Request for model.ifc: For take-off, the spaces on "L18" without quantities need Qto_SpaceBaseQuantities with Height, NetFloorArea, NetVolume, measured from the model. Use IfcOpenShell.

First a look at what the model holds.

```python
import ifcopenshell
import ifcopenshell.util.element
import ifcopenshell.util.unit

model = ifcopenshell.open("model.ifc")
print(model.schema)
for unit_type in ("LENGTHUNIT", "AREAUNIT", "VOLUMEUNIT"):
    print(unit_type, ifcopenshell.util.unit.calculate_unit_scale(model, unit_type))
storey = next(s for s in model.by_type("IfcBuildingStorey") if s.Name == "L18")
spaces = [e for e in ifcopenshell.util.element.get_decomposition(storey) if e.is_a("IfcSpace")]
for e in sorted(spaces, key=lambda e: e.id()):
    print(e.id(), e.is_a(), e.Name, list(ifcopenshell.util.element.get_psets(e, qtos_only=True)), sep=" | ")
```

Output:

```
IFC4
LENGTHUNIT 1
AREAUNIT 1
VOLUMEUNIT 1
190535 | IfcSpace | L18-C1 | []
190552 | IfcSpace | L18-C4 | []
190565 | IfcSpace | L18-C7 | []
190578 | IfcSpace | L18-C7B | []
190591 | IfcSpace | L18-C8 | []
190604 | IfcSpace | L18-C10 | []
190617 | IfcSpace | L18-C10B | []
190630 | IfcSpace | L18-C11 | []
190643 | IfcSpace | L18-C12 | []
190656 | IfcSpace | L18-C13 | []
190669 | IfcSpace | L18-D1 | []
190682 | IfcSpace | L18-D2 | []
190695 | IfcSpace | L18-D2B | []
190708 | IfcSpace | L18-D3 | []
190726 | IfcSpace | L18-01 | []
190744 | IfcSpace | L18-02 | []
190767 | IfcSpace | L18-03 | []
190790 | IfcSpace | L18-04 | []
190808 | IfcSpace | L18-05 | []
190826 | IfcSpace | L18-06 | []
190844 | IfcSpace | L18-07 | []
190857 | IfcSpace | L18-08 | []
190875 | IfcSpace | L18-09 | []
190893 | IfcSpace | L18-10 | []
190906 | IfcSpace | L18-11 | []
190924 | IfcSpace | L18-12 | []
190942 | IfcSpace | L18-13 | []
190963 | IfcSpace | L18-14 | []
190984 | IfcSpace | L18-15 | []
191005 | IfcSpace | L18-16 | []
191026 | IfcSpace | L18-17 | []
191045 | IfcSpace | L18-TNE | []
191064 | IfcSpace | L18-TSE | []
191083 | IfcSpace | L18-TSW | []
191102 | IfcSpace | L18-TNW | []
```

```python
import ifcopenshell
import ifcopenshell.api.pset
import ifcopenshell.geom
import ifcopenshell.util.element
import ifcopenshell.util.shape
import ifcopenshell.util.unit

model = ifcopenshell.open("model.ifc")
unit_scale = ifcopenshell.util.unit.calculate_unit_scale(model)
area_scale = ifcopenshell.util.unit.calculate_unit_scale(model, "AREAUNIT")
volume_scale = ifcopenshell.util.unit.calculate_unit_scale(model, "VOLUMEUNIT")
settings = ifcopenshell.geom.settings()

storey = next(s for s in model.by_type("IfcBuildingStorey") if s.Name == "L18")
spaces = [e for e in ifcopenshell.util.element.get_decomposition(storey) if e.is_a("IfcSpace")]

for e in sorted(spaces, key=lambda e: e.id()):
    if ifcopenshell.util.element.get_psets(e, qtos_only=True, should_inherit=False):
        continue
    # Geometry comes back in metres, in the element's own axes.
    shape = ifcopenshell.geom.create_shape(settings, e)
    values = {
        "Height": ifcopenshell.util.shape.get_z(shape.geometry) / unit_scale,
        "NetFloorArea": ifcopenshell.util.shape.get_footprint_area(shape.geometry) / area_scale,
        "NetVolume": ifcopenshell.util.shape.get_volume(shape.geometry) / volume_scale,
    }
    qto = ifcopenshell.api.pset.add_qto(model, product=e, name="Qto_SpaceBaseQuantities")
    ifcopenshell.api.pset.edit_qto(model, qto=qto, properties=values)
    print(e.id(), {k: round(v, 3) for k, v in values.items()})

model.write("model_rev.ifc")
```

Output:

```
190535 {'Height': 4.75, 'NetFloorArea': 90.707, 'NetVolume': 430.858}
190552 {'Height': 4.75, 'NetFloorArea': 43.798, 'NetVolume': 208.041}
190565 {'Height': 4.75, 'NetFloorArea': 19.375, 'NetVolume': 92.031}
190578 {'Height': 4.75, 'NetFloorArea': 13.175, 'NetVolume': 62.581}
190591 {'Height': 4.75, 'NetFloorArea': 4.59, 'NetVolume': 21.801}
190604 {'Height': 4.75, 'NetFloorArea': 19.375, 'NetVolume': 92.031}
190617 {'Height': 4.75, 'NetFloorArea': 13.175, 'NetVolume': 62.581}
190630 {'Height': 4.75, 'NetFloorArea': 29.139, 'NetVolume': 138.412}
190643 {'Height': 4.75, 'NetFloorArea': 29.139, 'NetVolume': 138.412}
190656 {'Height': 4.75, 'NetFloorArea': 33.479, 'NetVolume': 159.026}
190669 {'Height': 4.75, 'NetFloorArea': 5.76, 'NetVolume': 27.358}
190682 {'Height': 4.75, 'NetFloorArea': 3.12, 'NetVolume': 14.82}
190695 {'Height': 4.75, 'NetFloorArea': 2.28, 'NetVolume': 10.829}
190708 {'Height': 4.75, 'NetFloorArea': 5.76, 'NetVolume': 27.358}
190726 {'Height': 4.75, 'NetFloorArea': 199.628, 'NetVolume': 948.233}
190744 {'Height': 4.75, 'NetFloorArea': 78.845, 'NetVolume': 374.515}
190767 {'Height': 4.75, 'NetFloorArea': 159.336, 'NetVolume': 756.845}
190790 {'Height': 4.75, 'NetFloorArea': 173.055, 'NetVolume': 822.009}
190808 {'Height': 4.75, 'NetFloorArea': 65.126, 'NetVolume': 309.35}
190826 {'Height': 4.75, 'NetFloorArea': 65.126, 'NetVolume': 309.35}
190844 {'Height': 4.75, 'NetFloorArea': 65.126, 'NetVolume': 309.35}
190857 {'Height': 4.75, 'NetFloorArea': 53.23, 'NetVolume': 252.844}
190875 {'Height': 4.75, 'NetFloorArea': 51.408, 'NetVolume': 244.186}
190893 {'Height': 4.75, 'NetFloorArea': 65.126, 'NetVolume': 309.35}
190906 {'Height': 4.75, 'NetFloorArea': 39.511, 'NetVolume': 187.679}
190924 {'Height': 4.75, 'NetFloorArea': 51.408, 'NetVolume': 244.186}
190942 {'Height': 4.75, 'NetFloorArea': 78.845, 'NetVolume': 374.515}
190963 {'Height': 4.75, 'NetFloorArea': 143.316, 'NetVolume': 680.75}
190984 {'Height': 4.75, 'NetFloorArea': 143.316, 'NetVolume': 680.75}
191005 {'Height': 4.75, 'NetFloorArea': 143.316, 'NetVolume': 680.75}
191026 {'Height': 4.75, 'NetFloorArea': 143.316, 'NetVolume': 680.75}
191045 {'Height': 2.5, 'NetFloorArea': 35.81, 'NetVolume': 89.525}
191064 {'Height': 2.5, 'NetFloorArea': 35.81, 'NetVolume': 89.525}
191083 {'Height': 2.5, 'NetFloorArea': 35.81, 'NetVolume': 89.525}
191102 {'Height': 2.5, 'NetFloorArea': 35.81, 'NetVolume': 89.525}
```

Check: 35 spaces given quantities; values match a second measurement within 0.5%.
